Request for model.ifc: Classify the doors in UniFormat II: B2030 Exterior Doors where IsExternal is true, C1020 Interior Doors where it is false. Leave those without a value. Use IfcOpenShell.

First a look at what the model holds.

```python
import ifcopenshell
import ifcopenshell.util.element

model = ifcopenshell.open("model.ifc")
print(model.schema)
print("classifications:", [c.Name for c in model.by_type("IfcClassification")])
values = [ifcopenshell.util.element.get_pset(e, "Pset_DoorCommon", "IsExternal") for e in model.by_type("IfcDoor")]
for value in (True, False, None):
    print("IsExternal", value, values.count(value))
```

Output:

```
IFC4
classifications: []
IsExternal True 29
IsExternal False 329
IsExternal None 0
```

```python
import ifcopenshell
import ifcopenshell.api.classification
import ifcopenshell.util.element

model = ifcopenshell.open("model.ifc")

system = ifcopenshell.api.classification.add_classification(model, classification="UniFormat II")

doors = model.by_type("IfcDoor")
external = {e: ifcopenshell.util.element.get_pset(e, "Pset_DoorCommon", "IsExternal") for e in doors}
for flag, code, name in ((True, "B2030", "Exterior Doors"), (False, "C1020", "Interior Doors")):
    products = [e for e in doors if external[e] is flag]
    ifcopenshell.api.classification.add_reference(
        model, products=products, classification=system, identification=code, name=name
    )
    print(code, len(products))

model.write("model_rev.ifc")
```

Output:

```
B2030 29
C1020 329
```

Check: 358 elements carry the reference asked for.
